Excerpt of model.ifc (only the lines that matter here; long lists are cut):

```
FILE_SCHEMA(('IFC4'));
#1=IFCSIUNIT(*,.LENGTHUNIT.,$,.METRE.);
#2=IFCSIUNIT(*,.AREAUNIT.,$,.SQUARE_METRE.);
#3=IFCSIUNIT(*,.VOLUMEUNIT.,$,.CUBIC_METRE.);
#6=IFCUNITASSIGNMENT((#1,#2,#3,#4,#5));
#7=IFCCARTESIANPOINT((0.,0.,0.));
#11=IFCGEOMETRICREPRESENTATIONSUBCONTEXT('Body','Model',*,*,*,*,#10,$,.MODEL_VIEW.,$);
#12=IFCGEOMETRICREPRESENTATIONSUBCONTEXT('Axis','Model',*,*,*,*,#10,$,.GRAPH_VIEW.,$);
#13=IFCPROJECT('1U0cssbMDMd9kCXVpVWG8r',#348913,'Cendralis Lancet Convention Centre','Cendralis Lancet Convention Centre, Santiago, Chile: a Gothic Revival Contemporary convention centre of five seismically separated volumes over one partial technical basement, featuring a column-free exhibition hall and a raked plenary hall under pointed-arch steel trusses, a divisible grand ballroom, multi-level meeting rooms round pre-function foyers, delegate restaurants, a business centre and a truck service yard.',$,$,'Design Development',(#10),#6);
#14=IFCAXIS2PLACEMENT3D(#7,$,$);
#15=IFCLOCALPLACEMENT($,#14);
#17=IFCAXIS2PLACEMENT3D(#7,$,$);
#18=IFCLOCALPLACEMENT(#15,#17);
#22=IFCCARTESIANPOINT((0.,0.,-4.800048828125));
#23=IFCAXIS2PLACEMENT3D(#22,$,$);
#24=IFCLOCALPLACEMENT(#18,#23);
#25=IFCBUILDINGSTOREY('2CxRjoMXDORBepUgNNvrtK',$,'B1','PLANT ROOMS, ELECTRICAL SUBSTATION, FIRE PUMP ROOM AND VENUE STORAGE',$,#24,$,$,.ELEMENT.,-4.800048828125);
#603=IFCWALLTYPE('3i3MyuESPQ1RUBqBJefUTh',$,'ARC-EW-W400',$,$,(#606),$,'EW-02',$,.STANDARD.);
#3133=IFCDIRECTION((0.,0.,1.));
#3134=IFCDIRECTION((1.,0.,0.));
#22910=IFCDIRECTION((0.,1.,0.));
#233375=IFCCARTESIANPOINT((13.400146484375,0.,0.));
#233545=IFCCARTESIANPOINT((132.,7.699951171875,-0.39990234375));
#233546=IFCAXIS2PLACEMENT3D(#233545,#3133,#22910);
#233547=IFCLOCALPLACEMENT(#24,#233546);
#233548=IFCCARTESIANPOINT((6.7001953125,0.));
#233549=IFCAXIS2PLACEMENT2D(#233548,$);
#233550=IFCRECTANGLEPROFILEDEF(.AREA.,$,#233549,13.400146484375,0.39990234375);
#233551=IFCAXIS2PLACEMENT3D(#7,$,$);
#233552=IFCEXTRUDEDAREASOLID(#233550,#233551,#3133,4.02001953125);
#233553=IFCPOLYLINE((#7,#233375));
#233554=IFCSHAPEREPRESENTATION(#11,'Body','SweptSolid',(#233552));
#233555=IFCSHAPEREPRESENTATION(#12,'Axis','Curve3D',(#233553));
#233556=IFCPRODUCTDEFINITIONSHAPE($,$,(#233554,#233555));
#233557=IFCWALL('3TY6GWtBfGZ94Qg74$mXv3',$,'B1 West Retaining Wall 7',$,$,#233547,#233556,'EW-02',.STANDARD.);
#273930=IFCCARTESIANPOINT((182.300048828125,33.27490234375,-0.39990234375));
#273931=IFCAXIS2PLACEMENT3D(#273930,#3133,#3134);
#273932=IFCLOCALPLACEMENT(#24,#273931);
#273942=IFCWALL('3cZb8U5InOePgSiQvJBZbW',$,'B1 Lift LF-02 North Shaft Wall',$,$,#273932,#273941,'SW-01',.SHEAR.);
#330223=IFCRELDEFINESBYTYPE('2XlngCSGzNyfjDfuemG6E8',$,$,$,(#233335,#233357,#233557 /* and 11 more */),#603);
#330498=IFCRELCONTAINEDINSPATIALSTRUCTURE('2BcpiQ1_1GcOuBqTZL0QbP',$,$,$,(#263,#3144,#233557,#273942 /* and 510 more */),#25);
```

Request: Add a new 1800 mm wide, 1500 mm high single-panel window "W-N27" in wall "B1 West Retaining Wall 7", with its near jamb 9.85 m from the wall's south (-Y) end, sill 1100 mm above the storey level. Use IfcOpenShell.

```python
import numpy as np
import ifcopenshell
import ifcopenshell.api.feature
import ifcopenshell.api.geometry
import ifcopenshell.api.root
import ifcopenshell.api.spatial
import ifcopenshell.geom
import ifcopenshell.util.element
import ifcopenshell.util.placement
import ifcopenshell.util.representation
import ifcopenshell.util.shape
import ifcopenshell.util.unit

model = ifcopenshell.open("model.ifc")
unit_scale = ifcopenshell.util.unit.calculate_unit_scale(model)
settings = ifcopenshell.geom.settings()


def volume(element):
    """Net volume in cubic metres, openings subtracted."""
    shape = ifcopenshell.geom.create_shape(settings, element)
    return ifcopenshell.util.shape.get_volume(shape.geometry)


wall = model.by_id(233557)
storey = ifcopenshell.util.element.get_container(wall, ifc_class="IfcBuildingStorey")
context = ifcopenshell.util.representation.get_context(model, "Model", "Body", "MODEL_VIEW")
before = volume(wall)

width, height, from_end, sill = 1.8, 1.5, 9.85, 1.1  # metres

# The wall runs along its own X axis, and the end named is its -X end.
wall_shape = ifcopenshell.geom.create_shape(settings, wall)
x, y, z = ifcopenshell.util.shape.get_vertices(wall_shape.geometry).T
start = x.min() + from_end
face, thickness = float(y.min()), float(y.max() - y.min())
wall_matrix = ifcopenshell.util.placement.get_local_placement(wall.ObjectPlacement)
level = ifcopenshell.util.placement.get_local_placement(storey.ObjectPlacement)[2, 3]


def in_wall(x, y):
    """Placement at x, y metres in the wall's axes, at sill height."""
    matrix = wall_matrix.copy()
    matrix[:, 3] = wall_matrix @ np.array([x / unit_scale, y / unit_scale, 0.0, 1.0])
    matrix[2, 3] = level + sill / unit_scale
    return matrix


# Opening: a box that overshoots both wall faces by 50 mm.
opening = ifcopenshell.api.root.create_entity(model, ifc_class="IfcOpeningElement", predefined_type="OPENING")
box = ifcopenshell.api.geometry.add_wall_representation(
    model, context=context, length=width, height=height, thickness=thickness + 0.1
)
ifcopenshell.api.geometry.assign_representation(model, product=opening, representation=box)
ifcopenshell.api.geometry.edit_object_placement(model, product=opening, matrix=in_wall(start, face - 0.05), is_si=False)
ifcopenshell.api.feature.add_feature(model, feature=opening, element=wall)

window = ifcopenshell.api.root.create_entity(model, ifc_class="IfcWindow", name="W-N27", predefined_type="WINDOW")
window.OverallWidth, window.OverallHeight = width / unit_scale, height / unit_scale
window.PartitioningType = "SINGLE_PANEL"
body = ifcopenshell.api.geometry.add_window_representation(
    model,
    context=context,
    overall_width=window.OverallWidth,
    overall_height=window.OverallHeight,
    partition_type="SINGLE_PANEL",
)
ifcopenshell.api.geometry.assign_representation(model, product=window, representation=body)
ifcopenshell.api.spatial.assign_container(model, products=[window], relating_structure=storey)
ifcopenshell.api.feature.add_filling(model, opening=opening, element=window)

# Centre the window in the wall's thickness.
ifcopenshell.api.geometry.edit_object_placement(model, product=window, matrix=in_wall(start, face), is_si=False)
window_shape = ifcopenshell.geom.create_shape(settings, window)
depth = ifcopenshell.util.shape.get_vertices(window_shape.geometry)[:, 1]
offset = face + thickness / 2 - (depth.min() + depth.max()) / 2
ifcopenshell.api.geometry.edit_object_placement(model, product=window, matrix=in_wall(start, offset), is_si=False)

after = volume(wall)

print(f"wall volume {before:.3f} -> {after:.3f} m3")

model.write("model_rev.ifc")
```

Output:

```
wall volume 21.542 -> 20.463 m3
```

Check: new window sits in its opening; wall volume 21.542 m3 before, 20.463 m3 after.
